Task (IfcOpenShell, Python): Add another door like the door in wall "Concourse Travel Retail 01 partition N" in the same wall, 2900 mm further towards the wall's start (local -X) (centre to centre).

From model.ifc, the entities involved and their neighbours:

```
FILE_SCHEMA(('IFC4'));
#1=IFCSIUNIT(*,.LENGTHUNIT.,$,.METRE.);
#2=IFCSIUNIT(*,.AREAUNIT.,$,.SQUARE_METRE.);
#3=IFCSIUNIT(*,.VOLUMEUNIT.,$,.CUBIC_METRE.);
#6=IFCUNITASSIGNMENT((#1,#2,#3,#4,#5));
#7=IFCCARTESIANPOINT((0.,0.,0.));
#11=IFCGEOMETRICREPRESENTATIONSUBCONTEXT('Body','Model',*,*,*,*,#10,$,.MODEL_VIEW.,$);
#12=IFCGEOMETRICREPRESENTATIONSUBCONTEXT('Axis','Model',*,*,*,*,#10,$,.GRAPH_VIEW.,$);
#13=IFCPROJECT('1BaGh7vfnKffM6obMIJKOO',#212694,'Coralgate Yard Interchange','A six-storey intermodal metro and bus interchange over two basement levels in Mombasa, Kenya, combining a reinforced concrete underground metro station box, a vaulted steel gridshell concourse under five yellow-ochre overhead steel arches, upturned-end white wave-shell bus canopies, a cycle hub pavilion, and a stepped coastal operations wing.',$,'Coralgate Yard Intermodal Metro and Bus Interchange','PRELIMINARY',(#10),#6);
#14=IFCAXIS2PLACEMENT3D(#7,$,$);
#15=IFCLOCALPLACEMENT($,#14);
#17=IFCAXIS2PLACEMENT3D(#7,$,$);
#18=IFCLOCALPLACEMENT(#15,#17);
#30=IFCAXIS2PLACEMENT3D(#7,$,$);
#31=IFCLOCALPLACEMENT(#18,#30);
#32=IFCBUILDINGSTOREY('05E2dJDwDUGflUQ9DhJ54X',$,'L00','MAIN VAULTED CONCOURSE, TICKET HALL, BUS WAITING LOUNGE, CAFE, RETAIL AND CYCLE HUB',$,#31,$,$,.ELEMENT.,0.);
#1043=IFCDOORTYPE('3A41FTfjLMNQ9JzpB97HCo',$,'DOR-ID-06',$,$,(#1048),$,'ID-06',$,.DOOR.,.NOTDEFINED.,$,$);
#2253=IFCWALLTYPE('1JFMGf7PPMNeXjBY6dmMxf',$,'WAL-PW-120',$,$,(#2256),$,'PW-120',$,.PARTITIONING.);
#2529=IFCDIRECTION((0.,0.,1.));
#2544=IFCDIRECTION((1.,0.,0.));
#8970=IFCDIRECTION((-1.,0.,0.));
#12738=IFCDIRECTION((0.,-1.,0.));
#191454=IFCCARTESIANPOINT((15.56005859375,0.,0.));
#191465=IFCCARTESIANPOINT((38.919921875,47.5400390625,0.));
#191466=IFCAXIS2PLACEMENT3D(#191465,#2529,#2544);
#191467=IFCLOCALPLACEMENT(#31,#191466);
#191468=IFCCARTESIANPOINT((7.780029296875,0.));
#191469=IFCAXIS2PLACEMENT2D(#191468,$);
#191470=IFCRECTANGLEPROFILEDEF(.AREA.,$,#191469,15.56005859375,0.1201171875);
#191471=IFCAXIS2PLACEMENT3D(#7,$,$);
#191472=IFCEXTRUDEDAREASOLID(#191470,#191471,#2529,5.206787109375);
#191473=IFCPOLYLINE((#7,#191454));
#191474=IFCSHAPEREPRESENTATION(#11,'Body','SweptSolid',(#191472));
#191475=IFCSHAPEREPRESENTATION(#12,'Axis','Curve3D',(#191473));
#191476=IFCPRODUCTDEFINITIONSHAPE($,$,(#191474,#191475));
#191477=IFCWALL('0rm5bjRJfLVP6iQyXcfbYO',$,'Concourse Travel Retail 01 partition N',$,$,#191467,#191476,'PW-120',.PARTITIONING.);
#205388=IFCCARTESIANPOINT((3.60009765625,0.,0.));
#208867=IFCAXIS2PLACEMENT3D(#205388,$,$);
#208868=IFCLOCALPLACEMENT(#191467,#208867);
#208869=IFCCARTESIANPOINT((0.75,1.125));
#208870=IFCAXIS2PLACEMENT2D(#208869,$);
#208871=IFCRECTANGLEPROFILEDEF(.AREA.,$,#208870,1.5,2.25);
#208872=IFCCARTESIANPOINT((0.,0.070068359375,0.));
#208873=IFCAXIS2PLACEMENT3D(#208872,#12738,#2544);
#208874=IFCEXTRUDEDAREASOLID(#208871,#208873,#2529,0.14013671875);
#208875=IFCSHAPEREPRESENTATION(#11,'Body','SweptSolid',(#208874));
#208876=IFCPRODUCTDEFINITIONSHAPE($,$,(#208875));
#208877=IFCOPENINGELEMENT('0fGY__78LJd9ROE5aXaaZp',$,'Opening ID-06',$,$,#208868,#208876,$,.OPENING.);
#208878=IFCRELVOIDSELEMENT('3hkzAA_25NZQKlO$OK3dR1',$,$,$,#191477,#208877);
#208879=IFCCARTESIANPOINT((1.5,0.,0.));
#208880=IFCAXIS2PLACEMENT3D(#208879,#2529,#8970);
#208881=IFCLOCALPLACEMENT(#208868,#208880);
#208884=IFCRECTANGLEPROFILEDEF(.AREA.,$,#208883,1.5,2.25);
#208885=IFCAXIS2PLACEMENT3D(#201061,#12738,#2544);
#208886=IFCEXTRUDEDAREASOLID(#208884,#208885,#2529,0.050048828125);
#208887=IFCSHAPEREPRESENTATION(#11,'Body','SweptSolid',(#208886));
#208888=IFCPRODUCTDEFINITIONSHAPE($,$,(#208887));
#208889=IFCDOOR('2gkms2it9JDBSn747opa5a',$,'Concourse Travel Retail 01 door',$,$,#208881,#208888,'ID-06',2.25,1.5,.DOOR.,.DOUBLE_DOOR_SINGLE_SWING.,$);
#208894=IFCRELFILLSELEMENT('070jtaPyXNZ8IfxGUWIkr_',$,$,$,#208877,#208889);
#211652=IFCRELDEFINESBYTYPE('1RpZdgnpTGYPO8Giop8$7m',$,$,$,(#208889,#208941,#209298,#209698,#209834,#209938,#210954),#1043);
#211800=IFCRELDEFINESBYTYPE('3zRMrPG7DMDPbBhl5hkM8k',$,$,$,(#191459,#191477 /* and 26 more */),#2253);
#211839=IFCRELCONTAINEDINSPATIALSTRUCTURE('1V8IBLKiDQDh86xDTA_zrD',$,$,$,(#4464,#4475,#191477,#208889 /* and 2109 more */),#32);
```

```python
import ifcopenshell
import ifcopenshell.api.feature
import ifcopenshell.api.geometry
import ifcopenshell.api.root
import ifcopenshell.geom
import ifcopenshell.util.element
import ifcopenshell.util.placement
import ifcopenshell.util.shape

model = ifcopenshell.open("model.ifc")
settings = ifcopenshell.geom.settings()


def volume(element):
    """Net volume in cubic metres, openings subtracted."""
    shape = ifcopenshell.geom.create_shape(settings, element)
    return ifcopenshell.util.shape.get_volume(shape.geometry)


door = model.by_guid("2gkms2it9JDBSn747opa5a")
opening = door.FillsVoids[0].RelatingOpeningElement
wall = opening.VoidsElements[0].RelatingBuildingElement
before = volume(wall)
shift = ifcopenshell.util.placement.get_local_placement(wall.ObjectPlacement)[:3, 0] * -2.9

# copy_class copies the void relationship, type, container and properties, but no geometry.
new_opening = ifcopenshell.api.root.copy_class(model, product=opening)
new_opening.Representation = ifcopenshell.util.element.copy_deep(
    model, opening.Representation, exclude=["IfcGeometricRepresentationContext", "IfcRepresentationMap"]
)
new_door = ifcopenshell.api.root.copy_class(model, product=door)
new_door.Representation = ifcopenshell.util.element.copy_deep(
    model, door.Representation, exclude=["IfcGeometricRepresentationContext", "IfcRepresentationMap"]
)
new_door.Tag = None
ifcopenshell.api.feature.add_filling(model, opening=new_opening, element=new_door)

for old, new in ((opening, new_opening), (door, new_door)):
    matrix = ifcopenshell.util.placement.get_local_placement(old.ObjectPlacement)
    matrix[:3, 3] += shift
    ifcopenshell.api.geometry.edit_object_placement(model, product=new, matrix=matrix, is_si=False)

after = volume(wall)

print(f"wall volume {before:.3f} -> {after:.3f} m3")

model.write("model_edited.ifc")
```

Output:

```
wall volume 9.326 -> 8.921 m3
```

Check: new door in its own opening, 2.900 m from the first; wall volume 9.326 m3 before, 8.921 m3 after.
